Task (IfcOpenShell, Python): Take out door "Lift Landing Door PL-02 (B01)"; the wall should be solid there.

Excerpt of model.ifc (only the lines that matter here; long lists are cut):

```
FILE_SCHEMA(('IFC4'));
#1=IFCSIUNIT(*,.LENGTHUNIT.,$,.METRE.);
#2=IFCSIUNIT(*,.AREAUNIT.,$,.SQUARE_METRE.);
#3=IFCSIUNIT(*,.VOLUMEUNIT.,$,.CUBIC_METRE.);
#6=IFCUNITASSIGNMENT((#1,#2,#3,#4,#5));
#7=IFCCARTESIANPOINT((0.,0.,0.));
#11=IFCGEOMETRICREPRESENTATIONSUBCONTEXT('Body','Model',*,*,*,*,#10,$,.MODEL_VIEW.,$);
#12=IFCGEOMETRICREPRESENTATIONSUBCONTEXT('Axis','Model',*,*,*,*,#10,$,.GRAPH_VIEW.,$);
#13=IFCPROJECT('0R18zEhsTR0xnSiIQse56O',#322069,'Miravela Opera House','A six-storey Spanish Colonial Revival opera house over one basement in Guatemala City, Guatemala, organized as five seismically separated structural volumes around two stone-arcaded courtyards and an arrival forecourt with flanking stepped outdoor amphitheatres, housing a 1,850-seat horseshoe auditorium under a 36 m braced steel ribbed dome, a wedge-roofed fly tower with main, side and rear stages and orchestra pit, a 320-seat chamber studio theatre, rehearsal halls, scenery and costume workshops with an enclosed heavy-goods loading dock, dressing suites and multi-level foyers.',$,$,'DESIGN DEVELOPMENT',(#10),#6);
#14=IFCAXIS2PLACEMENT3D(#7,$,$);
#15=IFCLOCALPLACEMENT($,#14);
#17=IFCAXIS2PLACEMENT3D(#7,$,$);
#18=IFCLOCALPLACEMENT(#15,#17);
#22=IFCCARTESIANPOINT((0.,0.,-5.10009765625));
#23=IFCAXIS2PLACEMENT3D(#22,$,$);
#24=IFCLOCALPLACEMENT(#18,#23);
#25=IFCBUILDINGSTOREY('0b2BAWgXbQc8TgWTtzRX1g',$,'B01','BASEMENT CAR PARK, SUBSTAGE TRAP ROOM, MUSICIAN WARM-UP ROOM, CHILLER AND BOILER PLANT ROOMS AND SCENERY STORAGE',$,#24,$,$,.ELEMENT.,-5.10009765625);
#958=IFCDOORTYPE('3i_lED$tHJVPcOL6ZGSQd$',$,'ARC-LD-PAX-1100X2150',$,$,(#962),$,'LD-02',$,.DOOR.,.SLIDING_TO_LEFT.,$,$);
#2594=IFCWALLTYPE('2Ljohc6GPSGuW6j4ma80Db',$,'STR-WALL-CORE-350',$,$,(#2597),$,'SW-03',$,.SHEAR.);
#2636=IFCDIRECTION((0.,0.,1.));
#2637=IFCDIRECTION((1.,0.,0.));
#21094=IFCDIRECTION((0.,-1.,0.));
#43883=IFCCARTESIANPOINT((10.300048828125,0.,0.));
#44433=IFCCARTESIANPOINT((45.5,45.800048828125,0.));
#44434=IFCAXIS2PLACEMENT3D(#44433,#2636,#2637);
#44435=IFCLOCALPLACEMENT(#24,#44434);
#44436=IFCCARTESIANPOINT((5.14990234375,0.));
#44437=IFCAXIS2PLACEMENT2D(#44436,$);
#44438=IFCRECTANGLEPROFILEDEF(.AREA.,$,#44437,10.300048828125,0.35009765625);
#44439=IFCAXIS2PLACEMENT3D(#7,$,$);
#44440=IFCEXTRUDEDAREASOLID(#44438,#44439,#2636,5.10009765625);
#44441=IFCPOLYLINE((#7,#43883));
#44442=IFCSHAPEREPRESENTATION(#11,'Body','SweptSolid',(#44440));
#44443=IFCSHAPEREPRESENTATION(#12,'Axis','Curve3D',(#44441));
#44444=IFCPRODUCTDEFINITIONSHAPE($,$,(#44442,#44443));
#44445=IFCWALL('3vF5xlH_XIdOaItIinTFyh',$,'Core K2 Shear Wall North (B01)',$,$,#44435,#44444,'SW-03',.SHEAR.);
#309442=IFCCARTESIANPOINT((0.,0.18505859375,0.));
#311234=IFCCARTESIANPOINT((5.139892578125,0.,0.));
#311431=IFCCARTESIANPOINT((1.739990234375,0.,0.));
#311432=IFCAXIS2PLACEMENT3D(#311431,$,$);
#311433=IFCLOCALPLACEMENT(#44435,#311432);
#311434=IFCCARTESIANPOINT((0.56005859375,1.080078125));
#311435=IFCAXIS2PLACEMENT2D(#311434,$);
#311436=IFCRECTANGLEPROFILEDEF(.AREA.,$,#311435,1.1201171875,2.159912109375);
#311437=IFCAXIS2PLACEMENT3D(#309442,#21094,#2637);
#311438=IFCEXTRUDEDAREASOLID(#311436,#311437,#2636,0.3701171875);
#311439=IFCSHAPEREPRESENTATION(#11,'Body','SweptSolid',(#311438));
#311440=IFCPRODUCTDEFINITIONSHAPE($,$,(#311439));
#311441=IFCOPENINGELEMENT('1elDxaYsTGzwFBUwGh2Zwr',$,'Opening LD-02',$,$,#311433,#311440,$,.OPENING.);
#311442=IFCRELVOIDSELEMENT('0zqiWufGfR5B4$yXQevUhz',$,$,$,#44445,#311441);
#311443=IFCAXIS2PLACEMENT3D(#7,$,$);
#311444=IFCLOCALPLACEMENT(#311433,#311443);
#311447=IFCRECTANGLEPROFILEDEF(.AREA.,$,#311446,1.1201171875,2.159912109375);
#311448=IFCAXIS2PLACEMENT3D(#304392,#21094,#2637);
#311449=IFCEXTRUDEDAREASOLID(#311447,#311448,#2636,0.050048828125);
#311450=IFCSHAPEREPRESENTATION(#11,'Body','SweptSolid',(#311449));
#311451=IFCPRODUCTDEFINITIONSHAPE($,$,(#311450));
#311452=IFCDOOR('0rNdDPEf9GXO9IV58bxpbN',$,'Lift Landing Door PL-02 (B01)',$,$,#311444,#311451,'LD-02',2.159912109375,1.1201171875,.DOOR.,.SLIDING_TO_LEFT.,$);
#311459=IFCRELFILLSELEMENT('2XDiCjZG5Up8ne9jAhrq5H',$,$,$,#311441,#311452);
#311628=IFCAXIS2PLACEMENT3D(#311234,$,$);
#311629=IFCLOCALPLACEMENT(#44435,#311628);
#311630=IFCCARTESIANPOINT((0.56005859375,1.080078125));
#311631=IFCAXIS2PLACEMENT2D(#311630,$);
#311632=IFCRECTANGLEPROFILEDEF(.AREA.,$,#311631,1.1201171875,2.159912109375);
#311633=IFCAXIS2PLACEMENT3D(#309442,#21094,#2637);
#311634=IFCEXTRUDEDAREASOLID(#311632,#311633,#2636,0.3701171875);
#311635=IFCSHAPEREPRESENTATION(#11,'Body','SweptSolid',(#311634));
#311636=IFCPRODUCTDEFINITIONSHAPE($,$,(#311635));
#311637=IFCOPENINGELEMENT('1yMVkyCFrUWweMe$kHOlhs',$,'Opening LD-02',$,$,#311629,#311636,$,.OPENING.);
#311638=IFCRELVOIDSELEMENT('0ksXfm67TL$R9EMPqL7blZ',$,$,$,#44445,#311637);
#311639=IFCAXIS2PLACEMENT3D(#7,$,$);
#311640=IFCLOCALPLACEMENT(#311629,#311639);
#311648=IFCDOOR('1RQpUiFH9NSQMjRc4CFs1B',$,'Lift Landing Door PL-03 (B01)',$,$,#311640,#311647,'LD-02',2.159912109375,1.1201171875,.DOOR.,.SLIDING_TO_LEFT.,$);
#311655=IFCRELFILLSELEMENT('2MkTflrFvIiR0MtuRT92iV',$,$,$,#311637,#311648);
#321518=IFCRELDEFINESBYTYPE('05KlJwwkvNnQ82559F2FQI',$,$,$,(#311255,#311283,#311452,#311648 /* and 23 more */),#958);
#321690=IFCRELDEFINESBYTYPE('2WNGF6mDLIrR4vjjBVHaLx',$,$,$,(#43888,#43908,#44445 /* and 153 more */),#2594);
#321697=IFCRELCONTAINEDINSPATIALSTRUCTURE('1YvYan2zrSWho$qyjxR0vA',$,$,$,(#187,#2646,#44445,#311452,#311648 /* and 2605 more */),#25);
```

```python
import ifcopenshell
import ifcopenshell.api.feature
import ifcopenshell.api.root
import ifcopenshell.geom
import ifcopenshell.util.shape

model = ifcopenshell.open("model.ifc")
settings = ifcopenshell.geom.settings()


def volume(element):
    """Net volume in cubic metres, openings subtracted."""
    shape = ifcopenshell.geom.create_shape(settings, element)
    return ifcopenshell.util.shape.get_volume(shape.geometry)


door = model.by_guid("0rNdDPEf9GXO9IV58bxpbN")
opening = door.FillsVoids[0].RelatingOpeningElement
wall = opening.VoidsElements[0].RelatingBuildingElement
before = volume(wall)

ifcopenshell.api.root.remove_product(model, product=door)
ifcopenshell.api.feature.remove_feature(model, feature=opening)

after = volume(wall)

print(f"wall volume {before:.3f} -> {after:.3f} m3")

model.write("model_edited.ifc")
```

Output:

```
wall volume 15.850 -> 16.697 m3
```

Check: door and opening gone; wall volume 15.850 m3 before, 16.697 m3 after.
